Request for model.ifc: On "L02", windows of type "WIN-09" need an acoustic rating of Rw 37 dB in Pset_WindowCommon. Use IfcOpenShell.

First a look at what the model holds.

```python
import ifcopenshell
import ifcopenshell.util.element

model = ifcopenshell.open("model.ifc")
print(model.schema)
storey = next(s for s in model.by_type("IfcBuildingStorey") if s.Name == "L02")
windows = [e for e in ifcopenshell.util.element.get_decomposition(storey) if e.is_a("IfcWindow")]
seen = {}
for e in windows:
    element_type = ifcopenshell.util.element.get_type(e)
    key = (element_type.Name if element_type != e and element_type else None, ifcopenshell.util.element.get_pset(e, "Pset_WindowCommon", "AcousticRating"))
    seen[key] = seen.get(key, 0) + 1
for (name, value), count in sorted(seen.items(), key=str):
    print(count, "x", name, "|", value)
```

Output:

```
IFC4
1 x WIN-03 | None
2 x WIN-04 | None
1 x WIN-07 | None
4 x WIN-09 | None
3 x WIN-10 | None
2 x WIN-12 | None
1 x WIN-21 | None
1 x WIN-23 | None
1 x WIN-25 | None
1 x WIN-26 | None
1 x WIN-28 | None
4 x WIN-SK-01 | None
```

```python
import ifcopenshell
import ifcopenshell.api.pset
import ifcopenshell.util.element

model = ifcopenshell.open("model.ifc")

storey = next(s for s in model.by_type("IfcBuildingStorey") if s.Name == "L02")
windows = [e for e in ifcopenshell.util.element.get_decomposition(storey) if e.is_a("IfcWindow")]

count = 0
for e in windows:
    element_type = ifcopenshell.util.element.get_type(e)
    if element_type in (None, e) or element_type.Name != "WIN-09":
        continue
    # add_pset returns the element's existing set when there is one.
    pset = ifcopenshell.api.pset.add_pset(model, product=e, name="Pset_WindowCommon")
    ifcopenshell.api.pset.edit_pset(model, pset=pset, properties={"AcousticRating": "Rw 37 dB"})
    count += 1

print(count, "windows updated")

model.write("model_updated.ifc")
```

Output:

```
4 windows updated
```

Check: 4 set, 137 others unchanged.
